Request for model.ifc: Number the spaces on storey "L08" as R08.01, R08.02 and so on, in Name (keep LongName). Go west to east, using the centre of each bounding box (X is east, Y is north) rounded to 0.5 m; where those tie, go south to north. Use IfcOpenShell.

First a look at what the model holds.

```python
import ifcopenshell
import ifcopenshell.util.element
import ifcopenshell.util.placement

model = ifcopenshell.open("model.ifc")
print(model.schema)
storey = next(s for s in model.by_type("IfcBuildingStorey") if s.Name == "L08")
spaces = [e for e in ifcopenshell.util.element.get_decomposition(storey) if e.is_a("IfcSpace")]
for e in sorted(spaces, key=lambda e: e.id()):
    origin = ifcopenshell.util.placement.get_local_placement(e.ObjectPlacement)[:3, 3]
    print(e.id(), e.Name, e.LongName, origin.round(2) + 0.0, sep=" | ")
```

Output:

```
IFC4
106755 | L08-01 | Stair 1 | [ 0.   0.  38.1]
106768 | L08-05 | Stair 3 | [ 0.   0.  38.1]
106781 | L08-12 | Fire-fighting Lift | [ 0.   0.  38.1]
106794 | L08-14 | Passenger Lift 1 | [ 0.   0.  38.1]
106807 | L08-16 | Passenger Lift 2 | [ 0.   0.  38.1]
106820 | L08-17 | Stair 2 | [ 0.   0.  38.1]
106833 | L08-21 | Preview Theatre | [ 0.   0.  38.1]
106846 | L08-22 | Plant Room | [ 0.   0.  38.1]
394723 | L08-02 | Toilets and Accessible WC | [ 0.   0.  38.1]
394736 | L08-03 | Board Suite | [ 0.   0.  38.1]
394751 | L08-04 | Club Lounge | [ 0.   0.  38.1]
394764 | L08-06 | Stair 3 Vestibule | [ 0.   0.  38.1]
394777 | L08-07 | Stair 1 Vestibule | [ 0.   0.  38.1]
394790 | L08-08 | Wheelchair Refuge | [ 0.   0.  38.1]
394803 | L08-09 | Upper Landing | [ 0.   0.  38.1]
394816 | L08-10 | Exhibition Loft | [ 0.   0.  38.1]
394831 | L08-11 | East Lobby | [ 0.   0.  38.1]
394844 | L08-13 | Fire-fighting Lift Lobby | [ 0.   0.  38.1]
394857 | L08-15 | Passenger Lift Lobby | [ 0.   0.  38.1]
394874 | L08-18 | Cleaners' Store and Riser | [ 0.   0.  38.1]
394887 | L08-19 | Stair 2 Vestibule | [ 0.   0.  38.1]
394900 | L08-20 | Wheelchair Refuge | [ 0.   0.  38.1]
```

```python
import ifcopenshell
import ifcopenshell.geom
import ifcopenshell.util.element
import ifcopenshell.util.shape

model = ifcopenshell.open("model.ifc")
settings = ifcopenshell.geom.settings()
settings.set("use-world-coords", True)


def centre(element):
    shape = ifcopenshell.geom.create_shape(settings, element)
    return ifcopenshell.util.shape.get_bbox_centroid(shape.geometry)


storey = next(s for s in model.by_type("IfcBuildingStorey") if s.Name == "L08")
spaces = [e for e in ifcopenshell.util.element.get_decomposition(storey) if e.is_a("IfcSpace")]

# Insertion points can sit at a corner or the storey origin, so sort by the geometry (in metres).
centres = {e: centre(e) for e in spaces}
spaces.sort(key=lambda e: (round(centres[e][0] / 0.5), centres[e][1]))

for i, e in enumerate(spaces, start=1):
    number = f"R08.{i:02d}"
    e.Name = number
    print(e.id(), number)

model.write("model_rev.ifc")
```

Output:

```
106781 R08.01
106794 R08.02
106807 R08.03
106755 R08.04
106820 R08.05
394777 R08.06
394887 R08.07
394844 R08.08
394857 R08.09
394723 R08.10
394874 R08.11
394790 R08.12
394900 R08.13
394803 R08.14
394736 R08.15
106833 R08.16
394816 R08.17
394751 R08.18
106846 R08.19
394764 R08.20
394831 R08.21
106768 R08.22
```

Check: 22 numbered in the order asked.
